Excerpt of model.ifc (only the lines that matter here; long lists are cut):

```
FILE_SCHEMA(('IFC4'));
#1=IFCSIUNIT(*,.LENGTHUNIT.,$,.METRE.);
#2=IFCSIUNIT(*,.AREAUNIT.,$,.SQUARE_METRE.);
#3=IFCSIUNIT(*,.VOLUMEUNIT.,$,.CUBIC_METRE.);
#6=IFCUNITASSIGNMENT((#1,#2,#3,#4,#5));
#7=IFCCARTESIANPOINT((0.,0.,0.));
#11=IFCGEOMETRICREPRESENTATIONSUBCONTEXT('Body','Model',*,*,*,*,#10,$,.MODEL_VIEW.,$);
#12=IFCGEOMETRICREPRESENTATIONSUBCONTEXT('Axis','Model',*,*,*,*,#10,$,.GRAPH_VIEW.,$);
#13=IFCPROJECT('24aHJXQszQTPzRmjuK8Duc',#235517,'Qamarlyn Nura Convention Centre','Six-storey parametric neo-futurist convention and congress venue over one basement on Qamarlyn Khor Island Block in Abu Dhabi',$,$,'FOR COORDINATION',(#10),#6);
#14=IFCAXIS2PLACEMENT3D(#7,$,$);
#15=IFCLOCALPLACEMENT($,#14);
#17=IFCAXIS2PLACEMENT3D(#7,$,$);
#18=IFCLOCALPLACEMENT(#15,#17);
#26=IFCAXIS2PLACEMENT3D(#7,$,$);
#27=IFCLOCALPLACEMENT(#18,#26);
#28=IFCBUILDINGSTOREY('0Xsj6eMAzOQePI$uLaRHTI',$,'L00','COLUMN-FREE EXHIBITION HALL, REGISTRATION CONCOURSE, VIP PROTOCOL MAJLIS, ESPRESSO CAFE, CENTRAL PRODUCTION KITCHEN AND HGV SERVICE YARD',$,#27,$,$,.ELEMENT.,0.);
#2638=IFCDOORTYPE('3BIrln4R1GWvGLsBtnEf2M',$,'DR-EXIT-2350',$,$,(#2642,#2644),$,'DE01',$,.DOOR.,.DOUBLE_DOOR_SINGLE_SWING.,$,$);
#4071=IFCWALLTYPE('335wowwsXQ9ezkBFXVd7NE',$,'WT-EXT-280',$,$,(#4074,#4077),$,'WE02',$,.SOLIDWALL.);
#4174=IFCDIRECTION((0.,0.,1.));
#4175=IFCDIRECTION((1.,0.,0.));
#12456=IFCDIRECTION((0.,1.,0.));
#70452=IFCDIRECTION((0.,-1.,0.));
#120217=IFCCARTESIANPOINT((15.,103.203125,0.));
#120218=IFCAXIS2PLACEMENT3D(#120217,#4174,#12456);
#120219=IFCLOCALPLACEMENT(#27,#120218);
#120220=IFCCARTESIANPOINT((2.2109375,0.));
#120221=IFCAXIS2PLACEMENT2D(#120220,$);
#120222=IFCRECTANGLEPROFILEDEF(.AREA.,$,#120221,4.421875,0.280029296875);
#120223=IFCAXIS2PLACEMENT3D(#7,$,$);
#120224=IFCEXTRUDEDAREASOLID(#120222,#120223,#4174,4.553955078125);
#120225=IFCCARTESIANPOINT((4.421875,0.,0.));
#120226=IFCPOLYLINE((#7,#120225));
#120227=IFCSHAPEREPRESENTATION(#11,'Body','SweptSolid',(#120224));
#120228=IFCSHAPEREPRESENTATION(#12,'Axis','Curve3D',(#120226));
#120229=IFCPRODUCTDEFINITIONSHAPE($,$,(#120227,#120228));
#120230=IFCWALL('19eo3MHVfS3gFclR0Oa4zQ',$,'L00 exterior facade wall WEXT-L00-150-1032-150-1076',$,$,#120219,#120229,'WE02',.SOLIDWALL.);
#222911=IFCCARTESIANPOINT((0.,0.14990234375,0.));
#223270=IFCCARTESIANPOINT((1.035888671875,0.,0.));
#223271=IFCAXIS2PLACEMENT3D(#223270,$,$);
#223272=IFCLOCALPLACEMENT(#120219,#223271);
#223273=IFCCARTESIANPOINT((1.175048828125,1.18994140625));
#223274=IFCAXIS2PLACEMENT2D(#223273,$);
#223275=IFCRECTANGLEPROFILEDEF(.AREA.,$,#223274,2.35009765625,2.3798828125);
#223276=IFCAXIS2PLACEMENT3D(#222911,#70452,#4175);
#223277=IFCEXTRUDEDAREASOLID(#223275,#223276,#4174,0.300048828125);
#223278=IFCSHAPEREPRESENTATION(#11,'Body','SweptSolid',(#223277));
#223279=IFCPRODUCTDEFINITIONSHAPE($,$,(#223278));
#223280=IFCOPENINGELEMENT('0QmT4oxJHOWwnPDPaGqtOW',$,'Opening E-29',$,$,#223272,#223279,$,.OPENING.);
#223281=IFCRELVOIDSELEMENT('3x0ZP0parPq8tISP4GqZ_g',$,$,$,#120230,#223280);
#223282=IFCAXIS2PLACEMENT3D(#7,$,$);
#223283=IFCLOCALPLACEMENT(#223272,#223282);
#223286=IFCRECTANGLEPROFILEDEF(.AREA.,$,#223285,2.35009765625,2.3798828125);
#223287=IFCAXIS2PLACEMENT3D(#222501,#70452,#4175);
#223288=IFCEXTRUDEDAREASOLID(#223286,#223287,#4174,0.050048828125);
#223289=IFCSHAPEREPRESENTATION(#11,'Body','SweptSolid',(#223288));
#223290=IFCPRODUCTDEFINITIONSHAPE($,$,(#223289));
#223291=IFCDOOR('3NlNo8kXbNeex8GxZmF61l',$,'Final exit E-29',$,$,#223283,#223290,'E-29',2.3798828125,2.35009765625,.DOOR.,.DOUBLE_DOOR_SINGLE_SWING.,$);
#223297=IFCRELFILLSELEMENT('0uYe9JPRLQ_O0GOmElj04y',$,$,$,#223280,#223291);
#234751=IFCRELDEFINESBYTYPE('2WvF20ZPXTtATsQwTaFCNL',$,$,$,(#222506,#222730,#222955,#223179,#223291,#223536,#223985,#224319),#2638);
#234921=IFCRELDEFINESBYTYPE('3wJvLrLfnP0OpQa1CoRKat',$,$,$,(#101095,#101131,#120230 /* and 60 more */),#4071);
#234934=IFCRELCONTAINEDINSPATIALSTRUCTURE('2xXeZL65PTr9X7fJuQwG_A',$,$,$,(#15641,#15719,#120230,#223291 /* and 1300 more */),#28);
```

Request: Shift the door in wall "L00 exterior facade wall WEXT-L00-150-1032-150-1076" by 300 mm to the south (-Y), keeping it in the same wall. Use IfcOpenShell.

```python
import ifcopenshell
import ifcopenshell.api.geometry
import ifcopenshell.util.placement

model = ifcopenshell.open("model.ifc")

door = model.by_guid("3NlNo8kXbNeex8GxZmF61l")
opening = door.FillsVoids[0].RelatingOpeningElement
wall = opening.VoidsElements[0].RelatingBuildingElement

wall_matrix = ifcopenshell.util.placement.get_local_placement(wall.ObjectPlacement)
shift = wall_matrix[:3, 0] * -0.3
before = ifcopenshell.util.placement.get_local_placement(door.ObjectPlacement)[:3, 3].copy()

# The door is placed relative to its opening, so it follows when the opening moves.
matrix = ifcopenshell.util.placement.get_local_placement(opening.ObjectPlacement)
matrix[:3, 3] += shift
ifcopenshell.api.geometry.edit_object_placement(
    model, product=opening, matrix=matrix, is_si=False, should_transform_children=True
)

after = ifcopenshell.util.placement.get_local_placement(door.ObjectPlacement)[:3, 3]
print("door moved by", (after - before).round(3) + 0.0)

model.write("model_rev.ifc")
```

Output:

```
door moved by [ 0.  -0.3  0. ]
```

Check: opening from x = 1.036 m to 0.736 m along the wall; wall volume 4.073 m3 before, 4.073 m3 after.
